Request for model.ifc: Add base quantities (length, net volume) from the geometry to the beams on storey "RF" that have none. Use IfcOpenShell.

First a look at what the model holds.

```python
import ifcopenshell
import ifcopenshell.util.element
import ifcopenshell.util.unit

model = ifcopenshell.open("model.ifc")
print(model.schema)
for unit_type in ("LENGTHUNIT", "AREAUNIT", "VOLUMEUNIT"):
    print(unit_type, ifcopenshell.util.unit.calculate_unit_scale(model, unit_type))
storey = next(s for s in model.by_type("IfcBuildingStorey") if s.Name == "RF")
beams = [e for e in ifcopenshell.util.element.get_decomposition(storey) if e.is_a("IfcBeam")]
for e in sorted(beams, key=lambda e: e.id()):
    print(e.id(), e.is_a(), e.Name, list(ifcopenshell.util.element.get_psets(e, qtos_only=True)), sep=" | ")
```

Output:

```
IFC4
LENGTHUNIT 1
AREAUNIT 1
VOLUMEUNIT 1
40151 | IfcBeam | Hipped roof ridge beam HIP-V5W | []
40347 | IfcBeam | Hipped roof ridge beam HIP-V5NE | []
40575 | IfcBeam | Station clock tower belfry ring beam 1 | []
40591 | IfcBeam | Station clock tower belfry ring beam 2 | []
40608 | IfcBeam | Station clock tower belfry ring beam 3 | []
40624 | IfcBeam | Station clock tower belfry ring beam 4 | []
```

```python
import ifcopenshell
import ifcopenshell.api.pset
import ifcopenshell.geom
import ifcopenshell.util.element
import ifcopenshell.util.shape
import ifcopenshell.util.unit

model = ifcopenshell.open("model.ifc")
unit_scale = ifcopenshell.util.unit.calculate_unit_scale(model)
volume_scale = ifcopenshell.util.unit.calculate_unit_scale(model, "VOLUMEUNIT")
settings = ifcopenshell.geom.settings()

storey = next(s for s in model.by_type("IfcBuildingStorey") if s.Name == "RF")
beams = [e for e in ifcopenshell.util.element.get_decomposition(storey) if e.is_a("IfcBeam")]

for e in sorted(beams, key=lambda e: e.id()):
    if ifcopenshell.util.element.get_psets(e, qtos_only=True, should_inherit=False):
        continue
    # Geometry comes back in metres, in the element's own axes.
    shape = ifcopenshell.geom.create_shape(settings, e)
    values = {
        "Length": ifcopenshell.util.shape.get_max_xyz(shape.geometry) / unit_scale,
        "NetVolume": ifcopenshell.util.shape.get_volume(shape.geometry) / volume_scale,
    }
    qto = ifcopenshell.api.pset.add_qto(model, product=e, name="Qto_BeamBaseQuantities")
    ifcopenshell.api.pset.edit_qto(model, qto=qto, properties=values)
    print(e.id(), {k: round(v, 3) for k, v in values.items()})

model.write("model-out.ifc")
```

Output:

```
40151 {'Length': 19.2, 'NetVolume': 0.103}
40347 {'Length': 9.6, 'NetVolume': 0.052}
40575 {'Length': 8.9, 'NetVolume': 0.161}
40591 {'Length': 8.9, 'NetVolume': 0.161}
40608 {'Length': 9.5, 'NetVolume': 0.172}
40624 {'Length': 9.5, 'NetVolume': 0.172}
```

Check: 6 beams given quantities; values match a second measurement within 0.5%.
